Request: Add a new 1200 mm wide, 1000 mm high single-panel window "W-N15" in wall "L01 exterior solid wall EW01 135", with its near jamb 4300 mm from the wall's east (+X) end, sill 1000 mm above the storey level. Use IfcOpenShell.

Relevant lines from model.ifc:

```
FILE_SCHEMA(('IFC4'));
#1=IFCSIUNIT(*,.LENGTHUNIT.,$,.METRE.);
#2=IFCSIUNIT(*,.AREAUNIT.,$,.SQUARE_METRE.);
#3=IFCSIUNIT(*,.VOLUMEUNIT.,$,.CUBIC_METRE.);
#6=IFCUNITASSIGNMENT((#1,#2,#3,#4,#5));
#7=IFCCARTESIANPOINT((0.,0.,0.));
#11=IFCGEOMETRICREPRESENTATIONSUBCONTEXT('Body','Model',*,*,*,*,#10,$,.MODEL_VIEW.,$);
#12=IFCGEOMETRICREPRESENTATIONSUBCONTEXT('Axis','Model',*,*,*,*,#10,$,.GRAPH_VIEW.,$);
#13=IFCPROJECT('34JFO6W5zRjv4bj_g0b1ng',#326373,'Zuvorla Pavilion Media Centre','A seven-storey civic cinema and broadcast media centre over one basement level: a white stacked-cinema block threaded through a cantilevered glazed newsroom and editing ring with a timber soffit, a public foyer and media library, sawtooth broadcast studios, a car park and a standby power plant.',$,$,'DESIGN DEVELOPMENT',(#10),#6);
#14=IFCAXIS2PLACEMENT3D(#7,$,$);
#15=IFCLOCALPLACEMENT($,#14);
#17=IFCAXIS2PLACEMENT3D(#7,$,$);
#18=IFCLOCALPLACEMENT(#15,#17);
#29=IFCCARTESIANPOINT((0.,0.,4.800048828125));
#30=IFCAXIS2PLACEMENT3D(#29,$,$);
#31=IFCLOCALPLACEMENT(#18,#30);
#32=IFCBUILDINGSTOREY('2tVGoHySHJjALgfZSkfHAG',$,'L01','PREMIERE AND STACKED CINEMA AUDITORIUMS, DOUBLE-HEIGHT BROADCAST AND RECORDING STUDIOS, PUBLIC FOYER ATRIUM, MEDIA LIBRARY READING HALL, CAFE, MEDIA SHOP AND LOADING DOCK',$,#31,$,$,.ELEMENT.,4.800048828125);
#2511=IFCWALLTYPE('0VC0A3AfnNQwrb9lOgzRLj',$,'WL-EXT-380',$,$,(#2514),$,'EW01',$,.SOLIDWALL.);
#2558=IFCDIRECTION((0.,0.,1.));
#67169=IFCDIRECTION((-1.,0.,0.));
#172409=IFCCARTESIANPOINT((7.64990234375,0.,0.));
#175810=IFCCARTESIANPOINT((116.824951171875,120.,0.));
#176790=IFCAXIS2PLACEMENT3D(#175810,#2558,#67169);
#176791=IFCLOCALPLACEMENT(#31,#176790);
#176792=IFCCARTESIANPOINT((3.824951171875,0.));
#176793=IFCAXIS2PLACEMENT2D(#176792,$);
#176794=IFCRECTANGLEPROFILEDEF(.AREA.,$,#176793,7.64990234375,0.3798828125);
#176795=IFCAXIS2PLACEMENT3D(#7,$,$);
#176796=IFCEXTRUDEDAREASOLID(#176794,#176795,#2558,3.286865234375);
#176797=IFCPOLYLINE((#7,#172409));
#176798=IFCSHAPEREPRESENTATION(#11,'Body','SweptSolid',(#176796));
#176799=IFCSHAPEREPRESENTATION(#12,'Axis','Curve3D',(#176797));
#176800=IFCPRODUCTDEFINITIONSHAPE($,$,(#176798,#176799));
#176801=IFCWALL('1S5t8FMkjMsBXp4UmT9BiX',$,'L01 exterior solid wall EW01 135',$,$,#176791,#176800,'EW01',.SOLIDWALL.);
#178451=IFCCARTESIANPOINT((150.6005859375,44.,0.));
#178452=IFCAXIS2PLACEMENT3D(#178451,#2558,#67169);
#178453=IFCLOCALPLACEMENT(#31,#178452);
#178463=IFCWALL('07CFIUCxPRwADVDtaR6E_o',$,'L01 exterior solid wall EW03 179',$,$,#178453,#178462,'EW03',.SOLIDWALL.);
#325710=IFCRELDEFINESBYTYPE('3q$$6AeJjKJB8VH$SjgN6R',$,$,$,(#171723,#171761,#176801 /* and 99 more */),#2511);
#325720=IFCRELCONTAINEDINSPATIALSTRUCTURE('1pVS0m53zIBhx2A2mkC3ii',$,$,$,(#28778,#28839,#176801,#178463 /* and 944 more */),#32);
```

```python
import numpy as np
import ifcopenshell
import ifcopenshell.api.feature
import ifcopenshell.api.geometry
import ifcopenshell.api.root
import ifcopenshell.api.spatial
import ifcopenshell.geom
import ifcopenshell.util.element
import ifcopenshell.util.placement
import ifcopenshell.util.representation
import ifcopenshell.util.shape
import ifcopenshell.util.unit

model = ifcopenshell.open("model.ifc")
unit_scale = ifcopenshell.util.unit.calculate_unit_scale(model)
settings = ifcopenshell.geom.settings()


def volume(element):
    """Net volume in cubic metres, openings subtracted."""
    shape = ifcopenshell.geom.create_shape(settings, element)
    return ifcopenshell.util.shape.get_volume(shape.geometry)


wall = model.by_guid("1S5t8FMkjMsBXp4UmT9BiX")
storey = ifcopenshell.util.element.get_container(wall, ifc_class="IfcBuildingStorey")
context = ifcopenshell.util.representation.get_context(model, "Model", "Body", "MODEL_VIEW")
before = volume(wall)

width, height, from_end, sill = 1.2, 1, 4.3, 1  # metres

# The wall runs along its own X axis, and the end named is its -X end.
wall_shape = ifcopenshell.geom.create_shape(settings, wall)
x, y, z = ifcopenshell.util.shape.get_vertices(wall_shape.geometry).T
start = x.min() + from_end
face, thickness = float(y.min()), float(y.max() - y.min())
wall_matrix = ifcopenshell.util.placement.get_local_placement(wall.ObjectPlacement)
level = ifcopenshell.util.placement.get_local_placement(storey.ObjectPlacement)[2, 3]


def in_wall(x, y):
    """Placement at x, y metres in the wall's axes, at sill height."""
    matrix = wall_matrix.copy()
    matrix[:, 3] = wall_matrix @ np.array([x / unit_scale, y / unit_scale, 0.0, 1.0])
    matrix[2, 3] = level + sill / unit_scale
    return matrix


# Opening: a box that overshoots both wall faces by 50 mm.
opening = ifcopenshell.api.root.create_entity(model, ifc_class="IfcOpeningElement", predefined_type="OPENING")
box = ifcopenshell.api.geometry.add_wall_representation(
    model, context=context, length=width, height=height, thickness=thickness + 0.1
)
ifcopenshell.api.geometry.assign_representation(model, product=opening, representation=box)
ifcopenshell.api.geometry.edit_object_placement(model, product=opening, matrix=in_wall(start, face - 0.05), is_si=False)
ifcopenshell.api.feature.add_feature(model, feature=opening, element=wall)

window = ifcopenshell.api.root.create_entity(model, ifc_class="IfcWindow", name="W-N15", predefined_type="WINDOW")
window.OverallWidth, window.OverallHeight = width / unit_scale, height / unit_scale
window.PartitioningType = "SINGLE_PANEL"
body = ifcopenshell.api.geometry.add_window_representation(
    model,
    context=context,
    overall_width=window.OverallWidth,
    overall_height=window.OverallHeight,
    partition_type="SINGLE_PANEL",
)
ifcopenshell.api.geometry.assign_representation(model, product=window, representation=body)
ifcopenshell.api.spatial.assign_container(model, products=[window], relating_structure=storey)
ifcopenshell.api.feature.add_filling(model, opening=opening, element=window)

# Centre the window in the wall's thickness.
ifcopenshell.api.geometry.edit_object_placement(model, product=window, matrix=in_wall(start, face), is_si=False)
window_shape = ifcopenshell.geom.create_shape(settings, window)
depth = ifcopenshell.util.shape.get_vertices(window_shape.geometry)[:, 1]
offset = face + thickness / 2 - (depth.min() + depth.max()) / 2
ifcopenshell.api.geometry.edit_object_placement(model, product=window, matrix=in_wall(start, offset), is_si=False)

after = volume(wall)

print(f"wall volume {before:.3f} -> {after:.3f} m3")

model.write("model_updated.ifc")
```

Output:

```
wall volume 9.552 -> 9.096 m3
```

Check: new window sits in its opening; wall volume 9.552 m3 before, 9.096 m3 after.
